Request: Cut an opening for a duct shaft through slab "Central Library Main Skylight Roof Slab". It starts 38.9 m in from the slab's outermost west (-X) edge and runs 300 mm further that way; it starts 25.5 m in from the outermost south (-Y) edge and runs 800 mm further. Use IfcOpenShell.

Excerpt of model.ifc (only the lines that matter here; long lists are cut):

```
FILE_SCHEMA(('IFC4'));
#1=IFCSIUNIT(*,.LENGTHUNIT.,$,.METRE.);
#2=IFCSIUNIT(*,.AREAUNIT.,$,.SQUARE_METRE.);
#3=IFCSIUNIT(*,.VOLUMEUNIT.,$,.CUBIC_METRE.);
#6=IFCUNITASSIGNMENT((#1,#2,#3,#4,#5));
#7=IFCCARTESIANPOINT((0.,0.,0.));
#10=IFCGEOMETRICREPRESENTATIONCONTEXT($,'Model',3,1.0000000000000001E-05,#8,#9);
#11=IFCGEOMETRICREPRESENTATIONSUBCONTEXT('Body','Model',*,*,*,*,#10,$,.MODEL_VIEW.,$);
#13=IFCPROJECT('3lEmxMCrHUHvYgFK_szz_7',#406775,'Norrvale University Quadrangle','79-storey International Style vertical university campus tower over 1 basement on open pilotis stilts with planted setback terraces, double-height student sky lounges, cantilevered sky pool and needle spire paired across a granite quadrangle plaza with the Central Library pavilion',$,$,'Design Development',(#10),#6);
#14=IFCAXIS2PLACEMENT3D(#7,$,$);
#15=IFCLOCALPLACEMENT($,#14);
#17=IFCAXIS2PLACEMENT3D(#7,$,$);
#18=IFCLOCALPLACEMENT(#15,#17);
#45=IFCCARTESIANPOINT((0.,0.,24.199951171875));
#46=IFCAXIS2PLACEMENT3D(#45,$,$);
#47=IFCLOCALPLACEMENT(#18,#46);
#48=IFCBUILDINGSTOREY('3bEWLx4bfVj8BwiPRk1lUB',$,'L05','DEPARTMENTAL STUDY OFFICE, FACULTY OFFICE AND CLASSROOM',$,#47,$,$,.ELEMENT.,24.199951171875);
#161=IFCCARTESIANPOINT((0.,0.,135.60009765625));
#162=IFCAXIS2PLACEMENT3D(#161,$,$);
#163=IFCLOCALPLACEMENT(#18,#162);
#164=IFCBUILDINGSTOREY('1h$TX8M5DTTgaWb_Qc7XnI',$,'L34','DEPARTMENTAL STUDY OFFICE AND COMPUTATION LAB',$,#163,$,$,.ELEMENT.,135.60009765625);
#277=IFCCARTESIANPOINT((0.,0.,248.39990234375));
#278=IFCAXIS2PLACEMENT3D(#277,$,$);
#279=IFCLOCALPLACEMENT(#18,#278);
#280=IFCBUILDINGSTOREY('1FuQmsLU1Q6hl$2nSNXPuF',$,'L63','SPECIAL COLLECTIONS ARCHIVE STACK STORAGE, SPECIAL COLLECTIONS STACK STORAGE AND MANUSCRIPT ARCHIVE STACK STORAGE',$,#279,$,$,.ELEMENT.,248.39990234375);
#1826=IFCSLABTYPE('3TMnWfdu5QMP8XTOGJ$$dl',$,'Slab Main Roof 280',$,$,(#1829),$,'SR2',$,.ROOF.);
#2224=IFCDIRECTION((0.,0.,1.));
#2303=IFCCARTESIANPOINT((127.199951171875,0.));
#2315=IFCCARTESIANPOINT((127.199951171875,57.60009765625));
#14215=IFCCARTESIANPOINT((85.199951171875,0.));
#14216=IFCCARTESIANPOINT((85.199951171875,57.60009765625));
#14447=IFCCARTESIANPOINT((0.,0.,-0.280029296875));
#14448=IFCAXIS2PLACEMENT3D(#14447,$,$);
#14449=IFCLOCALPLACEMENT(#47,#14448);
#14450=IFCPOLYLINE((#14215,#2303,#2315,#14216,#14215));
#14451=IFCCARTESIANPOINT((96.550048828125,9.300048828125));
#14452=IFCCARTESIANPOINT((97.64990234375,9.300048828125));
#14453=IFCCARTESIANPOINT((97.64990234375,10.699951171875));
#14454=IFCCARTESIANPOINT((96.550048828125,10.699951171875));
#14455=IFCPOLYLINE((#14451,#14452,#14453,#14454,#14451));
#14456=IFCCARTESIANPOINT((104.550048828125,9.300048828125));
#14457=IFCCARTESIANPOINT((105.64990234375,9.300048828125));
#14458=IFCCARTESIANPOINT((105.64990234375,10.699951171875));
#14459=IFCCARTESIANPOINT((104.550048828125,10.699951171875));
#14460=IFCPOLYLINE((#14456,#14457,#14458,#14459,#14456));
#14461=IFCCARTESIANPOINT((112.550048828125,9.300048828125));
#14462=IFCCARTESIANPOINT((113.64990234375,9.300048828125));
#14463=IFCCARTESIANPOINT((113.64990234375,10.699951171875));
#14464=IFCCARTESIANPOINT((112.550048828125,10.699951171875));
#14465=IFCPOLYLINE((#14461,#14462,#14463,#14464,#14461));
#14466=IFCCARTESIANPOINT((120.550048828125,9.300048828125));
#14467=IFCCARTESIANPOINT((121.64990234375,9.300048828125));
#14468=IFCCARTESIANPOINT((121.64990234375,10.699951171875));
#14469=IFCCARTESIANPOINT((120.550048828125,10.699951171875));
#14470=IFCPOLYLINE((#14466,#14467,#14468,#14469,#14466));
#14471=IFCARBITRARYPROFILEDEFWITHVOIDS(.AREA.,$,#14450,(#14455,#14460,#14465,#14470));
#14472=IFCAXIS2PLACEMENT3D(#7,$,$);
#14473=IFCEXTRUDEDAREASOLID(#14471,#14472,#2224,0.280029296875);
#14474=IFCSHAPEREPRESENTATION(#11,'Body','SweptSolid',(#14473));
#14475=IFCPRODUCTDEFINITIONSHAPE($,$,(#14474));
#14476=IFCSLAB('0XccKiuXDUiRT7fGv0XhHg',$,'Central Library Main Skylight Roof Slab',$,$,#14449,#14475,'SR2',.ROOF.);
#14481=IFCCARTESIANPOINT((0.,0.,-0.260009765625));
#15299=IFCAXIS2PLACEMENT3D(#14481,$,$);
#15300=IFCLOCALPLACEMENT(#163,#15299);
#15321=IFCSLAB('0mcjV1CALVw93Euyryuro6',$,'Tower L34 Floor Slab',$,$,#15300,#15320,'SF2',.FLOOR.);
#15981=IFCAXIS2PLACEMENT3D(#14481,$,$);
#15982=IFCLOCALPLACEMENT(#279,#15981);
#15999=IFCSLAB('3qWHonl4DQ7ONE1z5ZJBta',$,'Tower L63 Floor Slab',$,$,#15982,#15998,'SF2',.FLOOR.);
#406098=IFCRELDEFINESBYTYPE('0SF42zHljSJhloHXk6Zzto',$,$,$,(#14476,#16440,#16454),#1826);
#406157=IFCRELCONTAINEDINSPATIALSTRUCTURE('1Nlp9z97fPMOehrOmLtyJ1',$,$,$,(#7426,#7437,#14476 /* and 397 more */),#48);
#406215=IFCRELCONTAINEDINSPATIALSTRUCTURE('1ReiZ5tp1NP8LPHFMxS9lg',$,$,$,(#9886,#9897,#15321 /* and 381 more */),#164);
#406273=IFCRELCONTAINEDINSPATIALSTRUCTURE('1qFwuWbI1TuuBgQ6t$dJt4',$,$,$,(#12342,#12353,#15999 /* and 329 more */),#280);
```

```python
import numpy as np
import ifcopenshell
import ifcopenshell.api.feature
import ifcopenshell.api.geometry
import ifcopenshell.api.root
import ifcopenshell.geom
import ifcopenshell.util.placement
import ifcopenshell.util.representation
import ifcopenshell.util.shape
import ifcopenshell.util.unit

model = ifcopenshell.open("model.ifc")
unit_scale = ifcopenshell.util.unit.calculate_unit_scale(model)
settings = ifcopenshell.geom.settings()


def volume(element):
    """Net volume in cubic metres, openings subtracted."""
    shape = ifcopenshell.geom.create_shape(settings, element)
    return ifcopenshell.util.shape.get_volume(shape.geometry)


slab = model.by_guid("0XccKiuXDUiRT7fGv0XhHg")
before = volume(slab)

# Extent in the slab's own axes, in metres. The edges named are its -X and -Y sides.
slab_shape = ifcopenshell.geom.create_shape(settings, slab)
vertices = ifcopenshell.util.shape.get_vertices(slab_shape.geometry)
x_min, y_min, bottom = vertices.min(axis=0)
top = vertices[:, 2].max()

opening = ifcopenshell.api.root.create_entity(model, ifc_class="IfcOpeningElement", name="Duct shaft opening", predefined_type="OPENING")
context = ifcopenshell.util.representation.get_context(model, "Model", "Body", "MODEL_VIEW")
width, depth = 0.3, 0.8
outline = [(0.0, 0.0), (width, 0.0), (width, depth), (0.0, depth), (0.0, 0.0)]
# Overshoot both faces by 50 mm so the cut is clean.
shape = ifcopenshell.api.geometry.add_slab_representation(
    model, context=context, depth=top - bottom + 0.1, polyline=outline
)
ifcopenshell.api.geometry.assign_representation(model, product=opening, representation=shape)

matrix = ifcopenshell.util.placement.get_local_placement(slab.ObjectPlacement)
matrix[:, 3] = matrix @ np.append(np.array([x_min + 38.9, y_min + 25.5, bottom - 0.05]) / unit_scale, 1.0)
ifcopenshell.api.geometry.edit_object_placement(model, product=opening, matrix=matrix, is_si=False)
ifcopenshell.api.feature.add_feature(model, feature=opening, element=slab)

after = volume(slab)

print(f"slab volume {before:.3f} -> {after:.3f} m3")

model.write("model_rev.ifc")
```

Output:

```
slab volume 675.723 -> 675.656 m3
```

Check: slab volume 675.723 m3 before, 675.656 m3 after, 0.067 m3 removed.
